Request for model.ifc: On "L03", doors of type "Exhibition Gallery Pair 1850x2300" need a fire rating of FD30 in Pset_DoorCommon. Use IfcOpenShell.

First a look at what the model holds.

```python
import ifcopenshell
import ifcopenshell.util.element

model = ifcopenshell.open("model.ifc")
print(model.schema)
storey = next(s for s in model.by_type("IfcBuildingStorey") if s.Name == "L03")
doors = [e for e in ifcopenshell.util.element.get_decomposition(storey) if e.is_a("IfcDoor")]
seen = {}
for e in doors:
    element_type = ifcopenshell.util.element.get_type(e)
    key = (element_type.Name if element_type != e and element_type else None, ifcopenshell.util.element.get_pset(e, "Pset_DoorCommon", "FireRating"))
    seen[key] = seen.get(key, 0) + 1
for (name, value), count in sorted(seen.items(), key=str):
    print(count, "x", name, "|", value)
```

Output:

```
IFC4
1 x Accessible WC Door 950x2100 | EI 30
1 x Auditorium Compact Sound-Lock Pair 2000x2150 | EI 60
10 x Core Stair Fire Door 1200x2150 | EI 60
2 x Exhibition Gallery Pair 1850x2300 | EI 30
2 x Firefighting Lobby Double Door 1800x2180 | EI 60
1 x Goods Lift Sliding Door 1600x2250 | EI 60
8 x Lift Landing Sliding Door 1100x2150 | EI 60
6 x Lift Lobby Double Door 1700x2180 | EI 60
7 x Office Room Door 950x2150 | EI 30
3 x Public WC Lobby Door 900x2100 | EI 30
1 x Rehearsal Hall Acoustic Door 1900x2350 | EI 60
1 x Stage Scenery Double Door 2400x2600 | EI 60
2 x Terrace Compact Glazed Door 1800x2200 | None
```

```python
import ifcopenshell
import ifcopenshell.api.pset
import ifcopenshell.util.element

model = ifcopenshell.open("model.ifc")

storey = next(s for s in model.by_type("IfcBuildingStorey") if s.Name == "L03")
doors = [e for e in ifcopenshell.util.element.get_decomposition(storey) if e.is_a("IfcDoor")]

count = 0
for e in doors:
    element_type = ifcopenshell.util.element.get_type(e)
    if element_type in (None, e) or element_type.Name != "Exhibition Gallery Pair 1850x2300":
        continue
    # add_pset returns the element's existing set when there is one.
    pset = ifcopenshell.api.pset.add_pset(model, product=e, name="Pset_DoorCommon")
    ifcopenshell.api.pset.edit_pset(model, pset=pset, properties={"FireRating": "FD30"})
    count += 1

print(count, "doors updated")

model.write("model_rev.ifc")
```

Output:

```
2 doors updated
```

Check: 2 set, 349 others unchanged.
